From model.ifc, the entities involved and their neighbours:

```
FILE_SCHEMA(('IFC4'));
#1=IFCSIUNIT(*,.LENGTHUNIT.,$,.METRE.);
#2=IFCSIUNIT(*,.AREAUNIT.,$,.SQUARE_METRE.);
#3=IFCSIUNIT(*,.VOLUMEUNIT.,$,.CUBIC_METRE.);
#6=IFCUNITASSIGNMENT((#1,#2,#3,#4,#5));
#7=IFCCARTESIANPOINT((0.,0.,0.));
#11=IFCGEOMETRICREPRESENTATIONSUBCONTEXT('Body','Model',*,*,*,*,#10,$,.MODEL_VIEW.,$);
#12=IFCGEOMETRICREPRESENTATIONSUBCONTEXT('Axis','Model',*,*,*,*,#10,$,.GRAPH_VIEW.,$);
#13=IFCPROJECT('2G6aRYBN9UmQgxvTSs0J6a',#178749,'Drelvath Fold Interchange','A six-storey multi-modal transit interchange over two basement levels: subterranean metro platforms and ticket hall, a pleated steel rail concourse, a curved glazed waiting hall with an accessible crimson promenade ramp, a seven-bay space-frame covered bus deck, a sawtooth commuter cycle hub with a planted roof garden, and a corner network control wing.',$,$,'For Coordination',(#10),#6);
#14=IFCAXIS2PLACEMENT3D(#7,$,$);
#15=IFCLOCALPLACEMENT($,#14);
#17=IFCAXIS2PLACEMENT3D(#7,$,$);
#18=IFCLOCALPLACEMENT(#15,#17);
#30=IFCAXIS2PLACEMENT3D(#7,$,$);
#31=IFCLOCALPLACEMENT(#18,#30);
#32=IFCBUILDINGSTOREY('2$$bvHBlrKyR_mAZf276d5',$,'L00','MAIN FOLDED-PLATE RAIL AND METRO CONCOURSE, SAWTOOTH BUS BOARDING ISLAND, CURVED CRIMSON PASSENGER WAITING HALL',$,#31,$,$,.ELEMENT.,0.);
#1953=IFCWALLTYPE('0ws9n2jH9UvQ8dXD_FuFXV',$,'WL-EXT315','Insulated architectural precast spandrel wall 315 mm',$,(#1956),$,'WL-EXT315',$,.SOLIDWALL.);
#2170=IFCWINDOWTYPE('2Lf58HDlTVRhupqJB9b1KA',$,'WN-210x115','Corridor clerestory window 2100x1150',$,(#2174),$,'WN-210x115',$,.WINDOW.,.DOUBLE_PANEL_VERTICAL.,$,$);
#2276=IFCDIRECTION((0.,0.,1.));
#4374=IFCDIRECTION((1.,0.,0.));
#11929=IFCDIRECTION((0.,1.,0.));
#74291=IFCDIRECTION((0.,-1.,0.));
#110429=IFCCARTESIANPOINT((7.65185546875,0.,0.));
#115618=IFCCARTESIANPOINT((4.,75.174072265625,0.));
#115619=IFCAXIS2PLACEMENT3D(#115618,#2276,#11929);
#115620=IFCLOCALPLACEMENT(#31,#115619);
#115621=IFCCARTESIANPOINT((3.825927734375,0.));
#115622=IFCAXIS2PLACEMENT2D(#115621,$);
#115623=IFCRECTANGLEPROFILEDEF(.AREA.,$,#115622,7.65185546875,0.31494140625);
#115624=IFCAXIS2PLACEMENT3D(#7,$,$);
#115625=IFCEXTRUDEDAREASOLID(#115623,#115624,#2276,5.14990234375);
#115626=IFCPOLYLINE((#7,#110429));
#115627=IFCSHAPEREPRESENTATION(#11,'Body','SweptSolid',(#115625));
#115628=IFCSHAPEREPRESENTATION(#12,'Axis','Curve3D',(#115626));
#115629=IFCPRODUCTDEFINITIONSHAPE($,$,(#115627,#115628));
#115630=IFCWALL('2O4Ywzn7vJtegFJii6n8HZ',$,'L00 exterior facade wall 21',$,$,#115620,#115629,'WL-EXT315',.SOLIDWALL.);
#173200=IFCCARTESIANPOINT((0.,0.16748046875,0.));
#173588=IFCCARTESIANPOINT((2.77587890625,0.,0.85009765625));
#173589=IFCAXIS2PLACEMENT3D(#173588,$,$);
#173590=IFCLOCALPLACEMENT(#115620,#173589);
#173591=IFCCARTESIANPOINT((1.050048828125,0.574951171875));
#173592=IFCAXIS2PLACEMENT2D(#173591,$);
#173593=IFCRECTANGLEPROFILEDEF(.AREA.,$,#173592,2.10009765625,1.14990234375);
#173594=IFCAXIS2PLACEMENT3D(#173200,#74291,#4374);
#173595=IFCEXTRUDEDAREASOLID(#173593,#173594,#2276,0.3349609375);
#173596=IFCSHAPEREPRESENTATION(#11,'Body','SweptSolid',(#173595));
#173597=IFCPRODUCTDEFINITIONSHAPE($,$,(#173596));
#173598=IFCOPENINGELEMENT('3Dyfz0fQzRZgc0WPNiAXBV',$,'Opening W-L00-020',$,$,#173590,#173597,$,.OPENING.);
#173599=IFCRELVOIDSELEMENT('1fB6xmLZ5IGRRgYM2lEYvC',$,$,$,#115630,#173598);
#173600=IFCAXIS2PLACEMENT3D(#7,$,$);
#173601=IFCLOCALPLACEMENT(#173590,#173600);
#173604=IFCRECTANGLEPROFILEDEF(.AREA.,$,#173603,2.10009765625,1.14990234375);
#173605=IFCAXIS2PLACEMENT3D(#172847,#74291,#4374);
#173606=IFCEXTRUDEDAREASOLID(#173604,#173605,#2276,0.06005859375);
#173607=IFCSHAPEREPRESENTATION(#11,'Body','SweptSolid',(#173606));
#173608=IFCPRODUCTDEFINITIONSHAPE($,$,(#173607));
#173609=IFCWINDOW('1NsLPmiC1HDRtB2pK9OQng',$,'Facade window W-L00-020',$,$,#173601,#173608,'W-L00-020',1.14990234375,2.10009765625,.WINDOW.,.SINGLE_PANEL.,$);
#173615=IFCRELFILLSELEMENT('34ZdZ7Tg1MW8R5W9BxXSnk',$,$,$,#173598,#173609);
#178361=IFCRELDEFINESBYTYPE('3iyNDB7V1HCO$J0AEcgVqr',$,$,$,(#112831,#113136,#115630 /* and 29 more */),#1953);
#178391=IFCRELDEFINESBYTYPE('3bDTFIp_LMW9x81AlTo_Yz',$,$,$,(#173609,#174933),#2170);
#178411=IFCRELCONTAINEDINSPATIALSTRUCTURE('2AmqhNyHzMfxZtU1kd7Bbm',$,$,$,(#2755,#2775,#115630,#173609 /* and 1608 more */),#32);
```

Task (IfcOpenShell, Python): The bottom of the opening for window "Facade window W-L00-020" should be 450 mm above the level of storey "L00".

```python
import numpy as np
import ifcopenshell
import ifcopenshell.api.geometry
import ifcopenshell.geom
import ifcopenshell.util.element
import ifcopenshell.util.placement
import ifcopenshell.util.shape
import ifcopenshell.util.unit

model = ifcopenshell.open("model.ifc")
unit_scale = ifcopenshell.util.unit.calculate_unit_scale(model)

window = model.by_guid("1NsLPmiC1HDRtB2pK9OQng")
opening = window.FillsVoids[0].RelatingOpeningElement
storey = ifcopenshell.util.element.get_container(window, ifc_class="IfcBuildingStorey")
level = ifcopenshell.util.placement.get_local_placement(storey.ObjectPlacement)[2, 3]

# The opening's origin need not be at the sill, so measure its lowest point.
shape = ifcopenshell.geom.create_shape(ifcopenshell.geom.settings(), opening)
bottom = ifcopenshell.util.shape.get_shape_bottom_elevation(shape, shape.geometry) / unit_scale
dz = level + 0.45 - bottom

shift = np.array([0.0, 0.0, dz])
# The window is placed relative to its opening, so it follows when the opening moves.
matrix = ifcopenshell.util.placement.get_local_placement(opening.ObjectPlacement)
matrix[:3, 3] += shift
ifcopenshell.api.geometry.edit_object_placement(
    model, product=opening, matrix=matrix, is_si=False, should_transform_children=True
)

print(f"moved by {dz * unit_scale:+.3f} m")

model.write("model_rev.ifc")
```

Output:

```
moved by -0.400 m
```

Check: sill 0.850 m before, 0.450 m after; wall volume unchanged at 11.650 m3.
